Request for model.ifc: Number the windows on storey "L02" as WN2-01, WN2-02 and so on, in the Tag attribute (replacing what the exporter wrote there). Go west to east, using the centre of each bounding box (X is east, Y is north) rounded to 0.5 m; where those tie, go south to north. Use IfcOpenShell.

First a look at what the model holds.

```python
import ifcopenshell
import ifcopenshell.util.element
import ifcopenshell.util.placement

model = ifcopenshell.open("model.ifc")
print(model.schema)
storey = next(s for s in model.by_type("IfcBuildingStorey") if s.Name == "L02")
windows = [e for e in ifcopenshell.util.element.get_decomposition(storey) if e.is_a("IfcWindow")]
for e in sorted(windows, key=lambda e: e.id()):
    origin = ifcopenshell.util.placement.get_local_placement(e.ObjectPlacement)[:3, 3]
    print(e.id(), e.Tag, e.Name, origin.round(2) + 0.0, sep=" | ")
```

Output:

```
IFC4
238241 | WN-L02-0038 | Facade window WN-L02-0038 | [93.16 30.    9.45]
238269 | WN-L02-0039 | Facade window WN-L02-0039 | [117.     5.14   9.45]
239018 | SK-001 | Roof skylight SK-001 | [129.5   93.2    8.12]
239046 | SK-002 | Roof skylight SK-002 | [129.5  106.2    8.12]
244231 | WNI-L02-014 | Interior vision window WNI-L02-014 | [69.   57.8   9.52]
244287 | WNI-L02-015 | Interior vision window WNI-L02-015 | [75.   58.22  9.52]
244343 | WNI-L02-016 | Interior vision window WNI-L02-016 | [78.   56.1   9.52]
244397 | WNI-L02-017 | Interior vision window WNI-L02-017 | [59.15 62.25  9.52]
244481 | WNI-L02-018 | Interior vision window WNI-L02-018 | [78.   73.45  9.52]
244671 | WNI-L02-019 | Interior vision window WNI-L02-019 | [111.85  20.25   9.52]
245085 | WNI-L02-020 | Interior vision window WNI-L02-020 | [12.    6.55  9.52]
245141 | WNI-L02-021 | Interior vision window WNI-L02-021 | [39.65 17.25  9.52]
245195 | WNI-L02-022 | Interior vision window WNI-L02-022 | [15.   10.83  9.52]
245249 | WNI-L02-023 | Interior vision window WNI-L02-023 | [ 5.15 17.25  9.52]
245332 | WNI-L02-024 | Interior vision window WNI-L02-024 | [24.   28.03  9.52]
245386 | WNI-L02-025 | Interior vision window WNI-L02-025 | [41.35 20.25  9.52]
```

```python
import ifcopenshell
import ifcopenshell.geom
import ifcopenshell.util.element
import ifcopenshell.util.shape

model = ifcopenshell.open("model.ifc")
settings = ifcopenshell.geom.settings()
settings.set("use-world-coords", True)


def centre(element):
    shape = ifcopenshell.geom.create_shape(settings, element)
    return ifcopenshell.util.shape.get_bbox_centroid(shape.geometry)


storey = next(s for s in model.by_type("IfcBuildingStorey") if s.Name == "L02")
windows = [e for e in ifcopenshell.util.element.get_decomposition(storey) if e.is_a("IfcWindow")]

# Insertion points can sit at a corner or the storey origin, so sort by the geometry (in metres).
centres = {e: centre(e) for e in windows}
windows.sort(key=lambda e: (round(centres[e][0] / 0.5), centres[e][1]))

for i, e in enumerate(windows, start=1):
    number = f"WN2-{i:02d}"
    e.Tag = number
    print(e.id(), number)

model.write("model_edited.ifc")
```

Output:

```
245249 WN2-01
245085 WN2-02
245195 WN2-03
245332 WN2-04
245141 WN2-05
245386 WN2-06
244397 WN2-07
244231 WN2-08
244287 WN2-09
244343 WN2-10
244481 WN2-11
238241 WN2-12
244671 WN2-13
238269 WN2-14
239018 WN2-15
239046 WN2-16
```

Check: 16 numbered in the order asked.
